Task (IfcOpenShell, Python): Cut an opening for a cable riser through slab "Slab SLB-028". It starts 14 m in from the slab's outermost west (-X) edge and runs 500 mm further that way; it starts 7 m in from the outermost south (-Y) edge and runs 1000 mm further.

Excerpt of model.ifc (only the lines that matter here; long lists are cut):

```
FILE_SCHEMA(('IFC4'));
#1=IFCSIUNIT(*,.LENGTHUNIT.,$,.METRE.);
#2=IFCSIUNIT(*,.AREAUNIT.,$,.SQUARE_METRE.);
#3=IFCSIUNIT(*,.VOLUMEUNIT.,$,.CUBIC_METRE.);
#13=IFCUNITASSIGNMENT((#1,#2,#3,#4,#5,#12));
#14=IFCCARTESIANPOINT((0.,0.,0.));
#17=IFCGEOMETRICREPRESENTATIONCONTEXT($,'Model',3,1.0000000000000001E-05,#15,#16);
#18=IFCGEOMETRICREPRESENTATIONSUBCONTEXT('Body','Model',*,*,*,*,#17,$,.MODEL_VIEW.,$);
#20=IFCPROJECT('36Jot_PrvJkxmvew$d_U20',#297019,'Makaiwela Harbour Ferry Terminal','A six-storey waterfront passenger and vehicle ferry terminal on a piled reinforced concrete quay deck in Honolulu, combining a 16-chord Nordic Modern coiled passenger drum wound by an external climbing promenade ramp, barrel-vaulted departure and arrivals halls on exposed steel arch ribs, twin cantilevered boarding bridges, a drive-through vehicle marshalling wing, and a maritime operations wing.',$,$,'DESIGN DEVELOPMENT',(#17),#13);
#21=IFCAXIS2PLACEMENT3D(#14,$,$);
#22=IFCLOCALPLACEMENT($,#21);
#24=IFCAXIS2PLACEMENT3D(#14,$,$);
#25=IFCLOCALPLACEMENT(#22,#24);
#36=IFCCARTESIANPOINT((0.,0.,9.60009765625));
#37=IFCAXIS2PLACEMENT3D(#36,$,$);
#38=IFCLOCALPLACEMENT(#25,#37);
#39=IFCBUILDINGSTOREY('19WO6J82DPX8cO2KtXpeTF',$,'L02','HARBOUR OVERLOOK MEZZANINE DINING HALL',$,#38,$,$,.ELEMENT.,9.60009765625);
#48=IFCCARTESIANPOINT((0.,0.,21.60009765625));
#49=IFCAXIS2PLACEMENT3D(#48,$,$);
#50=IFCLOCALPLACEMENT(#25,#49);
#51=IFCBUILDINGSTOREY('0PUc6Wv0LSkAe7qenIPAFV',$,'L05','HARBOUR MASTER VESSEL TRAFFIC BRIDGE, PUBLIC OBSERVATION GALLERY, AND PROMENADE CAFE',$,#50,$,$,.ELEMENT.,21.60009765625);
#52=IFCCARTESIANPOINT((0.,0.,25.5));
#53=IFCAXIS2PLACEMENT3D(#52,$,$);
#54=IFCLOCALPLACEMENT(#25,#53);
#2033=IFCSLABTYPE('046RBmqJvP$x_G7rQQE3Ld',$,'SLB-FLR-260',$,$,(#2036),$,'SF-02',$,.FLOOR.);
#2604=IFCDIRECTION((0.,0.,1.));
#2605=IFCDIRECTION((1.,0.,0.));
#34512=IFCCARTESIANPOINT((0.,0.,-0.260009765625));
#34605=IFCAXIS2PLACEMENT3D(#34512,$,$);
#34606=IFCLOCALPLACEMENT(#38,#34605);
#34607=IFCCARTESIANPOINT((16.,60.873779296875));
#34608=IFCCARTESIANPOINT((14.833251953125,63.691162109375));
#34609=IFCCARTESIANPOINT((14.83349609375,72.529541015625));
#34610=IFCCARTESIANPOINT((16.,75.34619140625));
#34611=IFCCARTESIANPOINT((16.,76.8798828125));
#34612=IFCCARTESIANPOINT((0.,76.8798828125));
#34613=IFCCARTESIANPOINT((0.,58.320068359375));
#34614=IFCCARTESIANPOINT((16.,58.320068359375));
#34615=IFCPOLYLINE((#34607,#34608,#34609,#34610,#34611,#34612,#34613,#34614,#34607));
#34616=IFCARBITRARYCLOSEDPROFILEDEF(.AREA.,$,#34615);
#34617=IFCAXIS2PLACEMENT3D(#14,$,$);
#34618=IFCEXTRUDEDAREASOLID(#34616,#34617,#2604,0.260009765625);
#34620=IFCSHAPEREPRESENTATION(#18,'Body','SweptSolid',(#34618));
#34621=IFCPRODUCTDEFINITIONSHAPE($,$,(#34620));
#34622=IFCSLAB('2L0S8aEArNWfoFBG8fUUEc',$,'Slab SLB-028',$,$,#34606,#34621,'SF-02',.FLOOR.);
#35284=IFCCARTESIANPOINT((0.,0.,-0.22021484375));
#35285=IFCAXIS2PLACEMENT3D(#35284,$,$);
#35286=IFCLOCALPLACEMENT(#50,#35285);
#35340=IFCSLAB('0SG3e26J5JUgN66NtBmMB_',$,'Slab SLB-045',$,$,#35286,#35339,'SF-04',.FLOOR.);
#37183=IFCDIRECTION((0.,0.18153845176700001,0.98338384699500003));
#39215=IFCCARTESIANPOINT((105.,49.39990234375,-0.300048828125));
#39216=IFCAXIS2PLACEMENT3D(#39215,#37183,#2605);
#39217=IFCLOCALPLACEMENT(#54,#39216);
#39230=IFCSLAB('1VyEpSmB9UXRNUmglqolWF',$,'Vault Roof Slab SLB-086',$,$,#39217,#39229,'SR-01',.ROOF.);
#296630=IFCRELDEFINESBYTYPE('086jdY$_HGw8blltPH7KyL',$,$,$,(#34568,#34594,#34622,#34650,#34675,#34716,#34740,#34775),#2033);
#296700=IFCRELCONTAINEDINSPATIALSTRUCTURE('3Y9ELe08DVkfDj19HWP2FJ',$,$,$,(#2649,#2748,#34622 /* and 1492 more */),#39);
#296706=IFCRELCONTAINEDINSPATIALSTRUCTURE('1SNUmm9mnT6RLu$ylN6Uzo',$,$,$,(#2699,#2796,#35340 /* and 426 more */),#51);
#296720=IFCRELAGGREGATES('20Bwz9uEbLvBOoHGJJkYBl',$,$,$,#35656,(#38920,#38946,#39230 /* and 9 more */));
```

```python
import numpy as np
import ifcopenshell
import ifcopenshell.api.feature
import ifcopenshell.api.geometry
import ifcopenshell.api.root
import ifcopenshell.geom
import ifcopenshell.util.placement
import ifcopenshell.util.representation
import ifcopenshell.util.shape
import ifcopenshell.util.unit

model = ifcopenshell.open("model.ifc")
unit_scale = ifcopenshell.util.unit.calculate_unit_scale(model)
settings = ifcopenshell.geom.settings()


def volume(element):
    """Net volume in cubic metres, openings subtracted."""
    shape = ifcopenshell.geom.create_shape(settings, element)
    return ifcopenshell.util.shape.get_volume(shape.geometry)


slab = model.by_guid("2L0S8aEArNWfoFBG8fUUEc")
before = volume(slab)

# Extent in the slab's own axes, in metres. The edges named are its -X and -Y sides.
slab_shape = ifcopenshell.geom.create_shape(settings, slab)
vertices = ifcopenshell.util.shape.get_vertices(slab_shape.geometry)
x_min, y_min, bottom = vertices.min(axis=0)
top = vertices[:, 2].max()

opening = ifcopenshell.api.root.create_entity(model, ifc_class="IfcOpeningElement", name="Cable riser opening", predefined_type="OPENING")
context = ifcopenshell.util.representation.get_context(model, "Model", "Body", "MODEL_VIEW")
width, depth = 0.5, 1
outline = [(0.0, 0.0), (width, 0.0), (width, depth), (0.0, depth), (0.0, 0.0)]
# Overshoot both faces by 50 mm so the cut is clean.
shape = ifcopenshell.api.geometry.add_slab_representation(
    model, context=context, depth=top - bottom + 0.1, polyline=outline
)
ifcopenshell.api.geometry.assign_representation(model, product=opening, representation=shape)

matrix = ifcopenshell.util.placement.get_local_placement(slab.ObjectPlacement)
matrix[:, 3] = matrix @ np.append(np.array([x_min + 14, y_min + 7, bottom - 0.05]) / unit_scale, 1.0)
ifcopenshell.api.geometry.edit_object_placement(model, product=opening, matrix=matrix, is_si=False)
ifcopenshell.api.feature.add_feature(model, feature=opening, element=slab)

after = volume(slab)

print(f"slab volume {before:.3f} -> {after:.3f} m3")

model.write("model-out.ifc")
```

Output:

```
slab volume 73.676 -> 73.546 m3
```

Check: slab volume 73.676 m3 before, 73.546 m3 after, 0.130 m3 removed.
